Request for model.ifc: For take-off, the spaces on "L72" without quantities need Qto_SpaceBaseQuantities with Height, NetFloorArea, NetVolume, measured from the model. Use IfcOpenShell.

First a look at what the model holds.

```python
import ifcopenshell
import ifcopenshell.util.element
import ifcopenshell.util.unit

model = ifcopenshell.open("model.ifc")
print(model.schema)
for unit_type in ("LENGTHUNIT", "AREAUNIT", "VOLUMEUNIT"):
    print(unit_type, ifcopenshell.util.unit.calculate_unit_scale(model, unit_type))
storey = next(s for s in model.by_type("IfcBuildingStorey") if s.Name == "L72")
spaces = [e for e in ifcopenshell.util.element.get_decomposition(storey) if e.is_a("IfcSpace")]
for e in sorted(spaces, key=lambda e: e.id()):
    print(e.id(), e.is_a(), e.Name, list(ifcopenshell.util.element.get_psets(e, qtos_only=True)), sep=" | ")
```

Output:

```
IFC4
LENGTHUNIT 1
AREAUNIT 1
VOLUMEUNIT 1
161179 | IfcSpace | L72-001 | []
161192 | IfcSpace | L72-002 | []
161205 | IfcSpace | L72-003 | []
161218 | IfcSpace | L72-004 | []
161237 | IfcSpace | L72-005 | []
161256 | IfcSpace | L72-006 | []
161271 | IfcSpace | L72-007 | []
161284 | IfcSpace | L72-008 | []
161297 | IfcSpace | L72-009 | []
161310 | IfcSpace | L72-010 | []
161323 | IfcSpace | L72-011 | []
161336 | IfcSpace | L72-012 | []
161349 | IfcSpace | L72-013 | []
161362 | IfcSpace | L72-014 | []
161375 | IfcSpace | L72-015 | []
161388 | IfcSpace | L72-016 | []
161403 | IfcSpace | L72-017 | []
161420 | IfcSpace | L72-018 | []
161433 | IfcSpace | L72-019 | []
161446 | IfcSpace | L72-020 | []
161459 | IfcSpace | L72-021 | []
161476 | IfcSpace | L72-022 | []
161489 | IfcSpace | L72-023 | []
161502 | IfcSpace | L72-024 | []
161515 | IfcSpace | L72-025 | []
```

```python
import ifcopenshell
import ifcopenshell.api.pset
import ifcopenshell.geom
import ifcopenshell.util.element
import ifcopenshell.util.shape
import ifcopenshell.util.unit

model = ifcopenshell.open("model.ifc")
unit_scale = ifcopenshell.util.unit.calculate_unit_scale(model)
area_scale = ifcopenshell.util.unit.calculate_unit_scale(model, "AREAUNIT")
volume_scale = ifcopenshell.util.unit.calculate_unit_scale(model, "VOLUMEUNIT")
settings = ifcopenshell.geom.settings()

storey = next(s for s in model.by_type("IfcBuildingStorey") if s.Name == "L72")
spaces = [e for e in ifcopenshell.util.element.get_decomposition(storey) if e.is_a("IfcSpace")]

for e in sorted(spaces, key=lambda e: e.id()):
    if ifcopenshell.util.element.get_psets(e, qtos_only=True, should_inherit=False):
        continue
    # Geometry comes back in metres, in the element's own axes.
    shape = ifcopenshell.geom.create_shape(settings, e)
    values = {
        "Height": ifcopenshell.util.shape.get_z(shape.geometry) / unit_scale,
        "NetFloorArea": ifcopenshell.util.shape.get_footprint_area(shape.geometry) / area_scale,
        "NetVolume": ifcopenshell.util.shape.get_volume(shape.geometry) / volume_scale,
    }
    qto = ifcopenshell.api.pset.add_qto(model, product=e, name="Qto_SpaceBaseQuantities")
    ifcopenshell.api.pset.edit_qto(model, qto=qto, properties=values)
    print(e.id(), {k: round(v, 3) for k, v in values.items()})

model.write("model_v2.ifc")
```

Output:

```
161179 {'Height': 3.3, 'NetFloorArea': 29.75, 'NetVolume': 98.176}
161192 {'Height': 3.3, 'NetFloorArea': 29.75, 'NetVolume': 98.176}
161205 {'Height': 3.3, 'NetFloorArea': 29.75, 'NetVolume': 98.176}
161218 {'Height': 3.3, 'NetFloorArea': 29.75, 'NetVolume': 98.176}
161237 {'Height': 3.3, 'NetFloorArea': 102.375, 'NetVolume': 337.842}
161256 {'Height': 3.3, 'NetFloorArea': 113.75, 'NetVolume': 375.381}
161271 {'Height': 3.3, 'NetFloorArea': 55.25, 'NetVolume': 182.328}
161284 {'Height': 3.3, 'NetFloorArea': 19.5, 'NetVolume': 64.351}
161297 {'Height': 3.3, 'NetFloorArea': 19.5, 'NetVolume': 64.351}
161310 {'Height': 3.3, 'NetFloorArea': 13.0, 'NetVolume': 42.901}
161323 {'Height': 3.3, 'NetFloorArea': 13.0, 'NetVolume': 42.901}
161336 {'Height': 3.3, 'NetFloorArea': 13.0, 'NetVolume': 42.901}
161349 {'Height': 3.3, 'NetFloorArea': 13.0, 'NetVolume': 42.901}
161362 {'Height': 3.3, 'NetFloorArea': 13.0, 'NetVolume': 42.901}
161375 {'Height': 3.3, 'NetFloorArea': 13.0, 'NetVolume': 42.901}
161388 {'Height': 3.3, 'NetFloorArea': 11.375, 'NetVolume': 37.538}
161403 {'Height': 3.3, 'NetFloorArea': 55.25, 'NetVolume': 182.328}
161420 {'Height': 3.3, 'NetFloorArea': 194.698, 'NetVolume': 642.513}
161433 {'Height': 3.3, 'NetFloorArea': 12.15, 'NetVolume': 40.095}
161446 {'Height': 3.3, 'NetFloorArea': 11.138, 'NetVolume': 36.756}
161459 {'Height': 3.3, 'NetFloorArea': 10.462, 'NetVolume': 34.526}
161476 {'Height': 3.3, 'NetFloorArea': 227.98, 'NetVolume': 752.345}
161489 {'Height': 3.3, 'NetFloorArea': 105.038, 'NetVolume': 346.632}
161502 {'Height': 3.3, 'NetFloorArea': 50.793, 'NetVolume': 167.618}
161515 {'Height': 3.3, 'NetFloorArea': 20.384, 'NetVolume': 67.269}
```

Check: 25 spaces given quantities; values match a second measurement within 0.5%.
